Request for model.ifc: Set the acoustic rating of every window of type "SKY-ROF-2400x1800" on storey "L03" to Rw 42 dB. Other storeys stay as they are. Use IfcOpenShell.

First a look at what the model holds.

```python
import ifcopenshell
import ifcopenshell.util.element

model = ifcopenshell.open("model.ifc")
print(model.schema)
storey = next(s for s in model.by_type("IfcBuildingStorey") if s.Name == "L03")
windows = [e for e in ifcopenshell.util.element.get_decomposition(storey) if e.is_a("IfcWindow")]
seen = {}
for e in windows:
    element_type = ifcopenshell.util.element.get_type(e)
    key = (element_type.Name if element_type != e and element_type else None, ifcopenshell.util.element.get_pset(e, "Pset_WindowCommon", "AcousticRating"))
    seen[key] = seen.get(key, 0) + 1
for (name, value), count in sorted(seen.items(), key=str):
    print(count, "x", name, "|", value)
```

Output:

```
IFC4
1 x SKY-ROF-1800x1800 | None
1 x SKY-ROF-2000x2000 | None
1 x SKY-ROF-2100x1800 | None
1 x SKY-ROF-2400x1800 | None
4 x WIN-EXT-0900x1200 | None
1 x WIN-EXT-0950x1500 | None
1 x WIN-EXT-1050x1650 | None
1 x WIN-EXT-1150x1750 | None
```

```python
import ifcopenshell
import ifcopenshell.api.pset
import ifcopenshell.util.element

model = ifcopenshell.open("model.ifc")

storey = next(s for s in model.by_type("IfcBuildingStorey") if s.Name == "L03")
windows = [e for e in ifcopenshell.util.element.get_decomposition(storey) if e.is_a("IfcWindow")]

count = 0
for e in windows:
    element_type = ifcopenshell.util.element.get_type(e)
    if element_type in (None, e) or element_type.Name != "SKY-ROF-2400x1800":
        continue
    # add_pset returns the element's existing set when there is one.
    pset = ifcopenshell.api.pset.add_pset(model, product=e, name="Pset_WindowCommon")
    ifcopenshell.api.pset.edit_pset(model, pset=pset, properties={"AcousticRating": "Rw 42 dB"})
    count += 1

print(count, "windows updated")

model.write("model_updated.ifc")
```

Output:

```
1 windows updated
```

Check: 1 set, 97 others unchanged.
